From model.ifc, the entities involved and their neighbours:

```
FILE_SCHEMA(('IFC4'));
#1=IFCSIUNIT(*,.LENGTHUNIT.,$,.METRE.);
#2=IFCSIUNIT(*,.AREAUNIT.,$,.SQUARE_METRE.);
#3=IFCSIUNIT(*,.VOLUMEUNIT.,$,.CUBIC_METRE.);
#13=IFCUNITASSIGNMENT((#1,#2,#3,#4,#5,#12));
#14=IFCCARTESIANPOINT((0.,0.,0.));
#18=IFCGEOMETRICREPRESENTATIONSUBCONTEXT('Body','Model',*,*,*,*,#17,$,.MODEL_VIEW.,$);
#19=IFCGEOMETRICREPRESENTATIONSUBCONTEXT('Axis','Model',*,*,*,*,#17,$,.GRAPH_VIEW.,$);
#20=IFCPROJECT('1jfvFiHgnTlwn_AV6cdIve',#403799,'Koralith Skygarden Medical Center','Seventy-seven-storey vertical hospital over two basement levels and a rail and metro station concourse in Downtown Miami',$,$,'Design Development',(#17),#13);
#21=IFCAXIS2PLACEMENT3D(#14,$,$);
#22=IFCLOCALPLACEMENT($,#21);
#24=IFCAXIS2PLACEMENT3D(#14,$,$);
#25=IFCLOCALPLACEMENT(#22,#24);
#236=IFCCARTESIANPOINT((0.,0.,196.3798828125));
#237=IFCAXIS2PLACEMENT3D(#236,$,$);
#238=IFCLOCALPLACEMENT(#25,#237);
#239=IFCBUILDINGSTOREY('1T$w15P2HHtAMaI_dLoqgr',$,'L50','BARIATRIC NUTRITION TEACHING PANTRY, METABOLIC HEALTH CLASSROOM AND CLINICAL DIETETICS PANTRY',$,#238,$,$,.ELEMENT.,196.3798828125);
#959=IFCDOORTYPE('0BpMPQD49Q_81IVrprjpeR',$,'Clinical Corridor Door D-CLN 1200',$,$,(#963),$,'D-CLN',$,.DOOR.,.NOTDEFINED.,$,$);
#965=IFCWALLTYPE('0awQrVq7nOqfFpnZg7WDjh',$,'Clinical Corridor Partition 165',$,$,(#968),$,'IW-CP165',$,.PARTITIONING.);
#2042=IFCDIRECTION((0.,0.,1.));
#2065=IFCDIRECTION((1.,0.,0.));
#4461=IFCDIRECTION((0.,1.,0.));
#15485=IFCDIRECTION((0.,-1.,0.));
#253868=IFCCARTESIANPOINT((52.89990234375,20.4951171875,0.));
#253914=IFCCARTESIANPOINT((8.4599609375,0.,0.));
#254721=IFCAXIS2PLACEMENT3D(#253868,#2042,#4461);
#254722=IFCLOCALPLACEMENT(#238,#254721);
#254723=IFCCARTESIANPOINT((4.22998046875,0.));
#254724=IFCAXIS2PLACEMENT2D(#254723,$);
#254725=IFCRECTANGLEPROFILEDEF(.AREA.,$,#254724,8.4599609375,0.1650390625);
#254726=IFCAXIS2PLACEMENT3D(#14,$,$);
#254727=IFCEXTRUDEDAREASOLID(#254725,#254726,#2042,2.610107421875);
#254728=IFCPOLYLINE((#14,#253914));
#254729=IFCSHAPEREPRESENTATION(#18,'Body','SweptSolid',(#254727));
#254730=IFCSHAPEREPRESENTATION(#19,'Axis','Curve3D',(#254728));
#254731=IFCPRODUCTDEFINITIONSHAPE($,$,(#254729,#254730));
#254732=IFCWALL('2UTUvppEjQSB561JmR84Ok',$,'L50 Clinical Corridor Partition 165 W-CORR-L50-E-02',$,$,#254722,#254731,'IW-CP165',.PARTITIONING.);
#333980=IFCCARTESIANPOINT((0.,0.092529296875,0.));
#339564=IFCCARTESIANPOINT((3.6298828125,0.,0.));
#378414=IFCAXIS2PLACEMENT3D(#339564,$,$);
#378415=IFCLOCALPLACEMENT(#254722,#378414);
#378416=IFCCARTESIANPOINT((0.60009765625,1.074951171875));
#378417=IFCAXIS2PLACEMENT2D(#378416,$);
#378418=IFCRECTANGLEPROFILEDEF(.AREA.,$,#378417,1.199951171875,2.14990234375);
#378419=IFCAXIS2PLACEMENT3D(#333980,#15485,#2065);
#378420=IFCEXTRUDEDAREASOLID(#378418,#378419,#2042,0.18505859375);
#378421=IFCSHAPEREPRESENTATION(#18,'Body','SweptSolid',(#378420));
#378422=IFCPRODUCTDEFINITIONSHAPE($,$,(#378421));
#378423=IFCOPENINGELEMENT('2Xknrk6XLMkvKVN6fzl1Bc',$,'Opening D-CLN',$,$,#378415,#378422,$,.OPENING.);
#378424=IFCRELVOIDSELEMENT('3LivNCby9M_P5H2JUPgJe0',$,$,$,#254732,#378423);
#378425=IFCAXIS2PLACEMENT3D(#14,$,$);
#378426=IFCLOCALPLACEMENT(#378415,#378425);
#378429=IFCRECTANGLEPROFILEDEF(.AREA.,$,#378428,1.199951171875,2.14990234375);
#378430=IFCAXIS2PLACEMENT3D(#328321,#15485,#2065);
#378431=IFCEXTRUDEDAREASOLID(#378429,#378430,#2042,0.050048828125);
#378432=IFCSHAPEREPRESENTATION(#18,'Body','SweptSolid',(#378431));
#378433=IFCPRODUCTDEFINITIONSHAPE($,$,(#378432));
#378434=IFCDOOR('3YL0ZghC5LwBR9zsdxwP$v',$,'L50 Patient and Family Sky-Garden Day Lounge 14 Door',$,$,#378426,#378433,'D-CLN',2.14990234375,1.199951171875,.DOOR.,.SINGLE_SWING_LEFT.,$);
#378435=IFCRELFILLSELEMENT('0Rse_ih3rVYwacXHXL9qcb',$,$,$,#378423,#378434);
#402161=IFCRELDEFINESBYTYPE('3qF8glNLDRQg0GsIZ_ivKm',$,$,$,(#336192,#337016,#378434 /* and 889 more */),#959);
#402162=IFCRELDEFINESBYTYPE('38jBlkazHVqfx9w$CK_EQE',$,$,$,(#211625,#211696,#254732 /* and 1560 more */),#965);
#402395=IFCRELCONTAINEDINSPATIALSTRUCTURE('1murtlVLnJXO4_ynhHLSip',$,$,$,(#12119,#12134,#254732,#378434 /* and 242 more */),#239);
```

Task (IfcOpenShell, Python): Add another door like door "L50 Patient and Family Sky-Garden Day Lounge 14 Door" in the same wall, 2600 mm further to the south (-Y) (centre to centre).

```python
import ifcopenshell
import ifcopenshell.api.feature
import ifcopenshell.api.geometry
import ifcopenshell.api.root
import ifcopenshell.geom
import ifcopenshell.util.element
import ifcopenshell.util.placement
import ifcopenshell.util.shape
import ifcopenshell.util.unit

model = ifcopenshell.open("model.ifc")
unit_scale = ifcopenshell.util.unit.calculate_unit_scale(model)
settings = ifcopenshell.geom.settings()


def volume(element):
    """Net volume in cubic metres, openings subtracted."""
    shape = ifcopenshell.geom.create_shape(settings, element)
    return ifcopenshell.util.shape.get_volume(shape.geometry)


door = model.by_guid("3YL0ZghC5LwBR9zsdxwP$v")
opening = door.FillsVoids[0].RelatingOpeningElement
wall = opening.VoidsElements[0].RelatingBuildingElement
before = volume(wall)
shift = ifcopenshell.util.placement.get_local_placement(wall.ObjectPlacement)[:3, 0] * -2.6 / unit_scale

# copy_class copies the void relationship, type, container and properties, but no geometry.
new_opening = ifcopenshell.api.root.copy_class(model, product=opening)
new_opening.Representation = ifcopenshell.util.element.copy_deep(
    model, opening.Representation, exclude=["IfcGeometricRepresentationContext", "IfcRepresentationMap"]
)
new_door = ifcopenshell.api.root.copy_class(model, product=door)
new_door.Representation = ifcopenshell.util.element.copy_deep(
    model, door.Representation, exclude=["IfcGeometricRepresentationContext", "IfcRepresentationMap"]
)
new_door.Tag = None
ifcopenshell.api.feature.add_filling(model, opening=new_opening, element=new_door)

for old, new in ((opening, new_opening), (door, new_door)):
    matrix = ifcopenshell.util.placement.get_local_placement(old.ObjectPlacement)
    matrix[:3, 3] += shift
    ifcopenshell.api.geometry.edit_object_placement(model, product=new, matrix=matrix, is_si=False)

after = volume(wall)

print(f"wall volume {before:.3f} -> {after:.3f} m3")

model.write("model_v2.ifc")
```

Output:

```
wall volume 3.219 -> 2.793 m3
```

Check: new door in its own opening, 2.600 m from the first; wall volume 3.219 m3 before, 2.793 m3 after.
